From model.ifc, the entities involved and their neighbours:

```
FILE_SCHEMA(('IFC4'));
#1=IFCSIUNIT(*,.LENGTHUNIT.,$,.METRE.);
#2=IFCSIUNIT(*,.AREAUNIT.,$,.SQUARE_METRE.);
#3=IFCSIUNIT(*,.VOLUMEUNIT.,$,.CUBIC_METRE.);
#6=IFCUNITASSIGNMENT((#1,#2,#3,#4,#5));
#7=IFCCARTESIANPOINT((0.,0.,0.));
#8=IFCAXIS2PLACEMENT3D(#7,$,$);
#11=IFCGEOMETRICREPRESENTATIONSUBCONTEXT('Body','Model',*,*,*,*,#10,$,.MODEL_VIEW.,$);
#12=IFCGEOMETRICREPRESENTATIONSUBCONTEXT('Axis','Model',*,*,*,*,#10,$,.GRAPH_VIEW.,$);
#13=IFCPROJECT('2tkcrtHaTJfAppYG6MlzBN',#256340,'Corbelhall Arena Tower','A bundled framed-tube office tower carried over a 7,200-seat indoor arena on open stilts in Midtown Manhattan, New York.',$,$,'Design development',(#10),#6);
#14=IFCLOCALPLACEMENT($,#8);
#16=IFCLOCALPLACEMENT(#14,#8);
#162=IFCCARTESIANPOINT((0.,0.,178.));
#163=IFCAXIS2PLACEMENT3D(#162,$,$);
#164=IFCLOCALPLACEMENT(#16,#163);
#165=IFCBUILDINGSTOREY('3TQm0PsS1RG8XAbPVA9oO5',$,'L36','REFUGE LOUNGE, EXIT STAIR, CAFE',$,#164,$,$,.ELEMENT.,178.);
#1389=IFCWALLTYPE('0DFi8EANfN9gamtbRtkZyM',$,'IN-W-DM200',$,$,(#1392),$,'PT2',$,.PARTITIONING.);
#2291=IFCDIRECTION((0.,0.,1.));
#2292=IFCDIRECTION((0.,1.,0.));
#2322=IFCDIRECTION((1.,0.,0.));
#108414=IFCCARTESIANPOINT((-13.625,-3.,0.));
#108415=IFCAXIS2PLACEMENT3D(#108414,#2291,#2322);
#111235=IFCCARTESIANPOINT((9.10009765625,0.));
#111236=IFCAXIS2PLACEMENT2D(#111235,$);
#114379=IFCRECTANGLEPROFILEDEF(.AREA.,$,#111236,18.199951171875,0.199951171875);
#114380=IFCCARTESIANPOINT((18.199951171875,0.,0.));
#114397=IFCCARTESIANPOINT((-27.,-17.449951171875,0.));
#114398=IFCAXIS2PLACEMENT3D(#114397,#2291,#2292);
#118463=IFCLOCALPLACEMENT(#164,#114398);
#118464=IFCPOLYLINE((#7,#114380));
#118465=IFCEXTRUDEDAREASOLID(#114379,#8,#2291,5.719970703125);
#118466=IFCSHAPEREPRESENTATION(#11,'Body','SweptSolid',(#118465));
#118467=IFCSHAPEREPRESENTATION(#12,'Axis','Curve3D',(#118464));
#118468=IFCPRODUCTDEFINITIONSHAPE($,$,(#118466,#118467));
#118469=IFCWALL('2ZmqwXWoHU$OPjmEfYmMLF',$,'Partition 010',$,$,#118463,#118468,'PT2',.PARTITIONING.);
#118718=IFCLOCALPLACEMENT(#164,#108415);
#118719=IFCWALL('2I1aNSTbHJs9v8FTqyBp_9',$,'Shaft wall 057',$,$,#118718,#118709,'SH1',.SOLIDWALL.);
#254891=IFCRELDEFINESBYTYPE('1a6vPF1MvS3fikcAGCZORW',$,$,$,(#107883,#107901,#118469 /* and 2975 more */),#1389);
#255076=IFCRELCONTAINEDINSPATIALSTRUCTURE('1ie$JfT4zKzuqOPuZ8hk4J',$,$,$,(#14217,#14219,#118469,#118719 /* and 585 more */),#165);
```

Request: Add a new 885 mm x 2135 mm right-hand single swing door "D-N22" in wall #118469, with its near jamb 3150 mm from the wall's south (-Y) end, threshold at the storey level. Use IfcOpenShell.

```python
import numpy as np
import ifcopenshell
import ifcopenshell.api.feature
import ifcopenshell.api.geometry
import ifcopenshell.api.root
import ifcopenshell.api.spatial
import ifcopenshell.geom
import ifcopenshell.util.element
import ifcopenshell.util.placement
import ifcopenshell.util.representation
import ifcopenshell.util.shape
import ifcopenshell.util.unit

model = ifcopenshell.open("model.ifc")
unit_scale = ifcopenshell.util.unit.calculate_unit_scale(model)
settings = ifcopenshell.geom.settings()


def volume(element):
    """Net volume in cubic metres, openings subtracted."""
    shape = ifcopenshell.geom.create_shape(settings, element)
    return ifcopenshell.util.shape.get_volume(shape.geometry)


wall = model.by_guid("2ZmqwXWoHU$OPjmEfYmMLF")
storey = ifcopenshell.util.element.get_container(wall, ifc_class="IfcBuildingStorey")
context = ifcopenshell.util.representation.get_context(model, "Model", "Body", "MODEL_VIEW")
before = volume(wall)

width, height, from_end, sill = 0.885, 2.135, 3.15, 0.0  # metres

# The wall runs along its own X axis, and the end named is its -X end.
wall_shape = ifcopenshell.geom.create_shape(settings, wall)
x, y, z = ifcopenshell.util.shape.get_vertices(wall_shape.geometry).T
start = x.min() + from_end
face, thickness = float(y.min()), float(y.max() - y.min())
wall_matrix = ifcopenshell.util.placement.get_local_placement(wall.ObjectPlacement)
level = ifcopenshell.util.placement.get_local_placement(storey.ObjectPlacement)[2, 3]


def in_wall(x, y):
    """Placement at x, y metres in the wall's axes, at sill height."""
    matrix = wall_matrix.copy()
    matrix[:, 3] = wall_matrix @ np.array([x / unit_scale, y / unit_scale, 0.0, 1.0])
    matrix[2, 3] = level + sill / unit_scale
    return matrix


# Opening: a box that overshoots both wall faces by 50 mm.
opening = ifcopenshell.api.root.create_entity(model, ifc_class="IfcOpeningElement", predefined_type="OPENING")
box = ifcopenshell.api.geometry.add_wall_representation(
    model, context=context, length=width, height=height, thickness=thickness + 0.1
)
ifcopenshell.api.geometry.assign_representation(model, product=opening, representation=box)
ifcopenshell.api.geometry.edit_object_placement(model, product=opening, matrix=in_wall(start, face - 0.05), is_si=False)
ifcopenshell.api.feature.add_feature(model, feature=opening, element=wall)

door = ifcopenshell.api.root.create_entity(model, ifc_class="IfcDoor", name="D-N22", predefined_type="DOOR")
door.OverallWidth, door.OverallHeight = width / unit_scale, height / unit_scale
door.OperationType = "SINGLE_SWING_RIGHT"
body = ifcopenshell.api.geometry.add_door_representation(
    model,
    context=context,
    overall_width=door.OverallWidth,
    overall_height=door.OverallHeight,
    operation_type="SINGLE_SWING_RIGHT",
    lining_properties={"LiningDepth": thickness / unit_scale, "ThresholdDepth": thickness / unit_scale},
)
ifcopenshell.api.geometry.assign_representation(model, product=door, representation=body)
ifcopenshell.api.spatial.assign_container(model, products=[door], relating_structure=storey)
ifcopenshell.api.feature.add_filling(model, opening=opening, element=door)

# The lining spans the wall, so the door starts at the wall face.
ifcopenshell.api.geometry.edit_object_placement(model, product=door, matrix=in_wall(start, face), is_si=False)

after = volume(wall)

print(f"wall volume {before:.3f} -> {after:.3f} m3")

model.write("model_rev.ifc")
```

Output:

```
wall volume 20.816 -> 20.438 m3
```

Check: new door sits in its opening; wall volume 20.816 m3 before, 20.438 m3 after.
